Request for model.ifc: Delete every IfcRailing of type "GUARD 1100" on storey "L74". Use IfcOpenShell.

First a look at what the model holds.

```python
import ifcopenshell
import ifcopenshell.util.element

model = ifcopenshell.open("model.ifc")
print(model.schema)
storey = next(s for s in model.by_type("IfcBuildingStorey") if s.Name == "L74")
railings = [e for e in ifcopenshell.util.element.get_decomposition(storey) if e.is_a("IfcRailing")]
seen = {}
for e in railings:
    element_type = ifcopenshell.util.element.get_type(e)
    name = element_type.Name if element_type not in (None, e) else None
    seen[name] = seen.get(name, 0) + 1
for name, count in sorted(seen.items(), key=str):
    print(count, "x", name)
```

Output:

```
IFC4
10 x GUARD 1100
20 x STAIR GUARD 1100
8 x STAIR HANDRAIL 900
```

```python
import ifcopenshell
import ifcopenshell.api.root
import ifcopenshell.util.element

model = ifcopenshell.open("model.ifc")

storey = next(s for s in model.by_type("IfcBuildingStorey") if s.Name == "L74")
railings = [e for e in ifcopenshell.util.element.get_decomposition(storey) if e.is_a("IfcRailing")]
targets = [e for e in railings if (t := ifcopenshell.util.element.get_type(e)) not in (None, e) and t.Name == "GUARD 1100"]

for e in targets:
    ifcopenshell.api.root.remove_product(model, product=e)
print(len(targets), "removed")

model.write("model_edited.ifc")
```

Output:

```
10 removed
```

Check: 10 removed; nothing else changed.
